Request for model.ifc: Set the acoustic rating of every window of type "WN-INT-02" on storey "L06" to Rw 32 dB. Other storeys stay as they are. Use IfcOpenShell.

First a look at what the model holds.

```python
import ifcopenshell
import ifcopenshell.util.element

model = ifcopenshell.open("model.ifc")
print(model.schema)
storey = next(s for s in model.by_type("IfcBuildingStorey") if s.Name == "L06")
windows = [e for e in ifcopenshell.util.element.get_decomposition(storey) if e.is_a("IfcWindow")]
seen = {}
for e in windows:
    element_type = ifcopenshell.util.element.get_type(e)
    key = (element_type.Name if element_type != e and element_type else None, ifcopenshell.util.element.get_pset(e, "Pset_WindowCommon", "AcousticRating"))
    seen[key] = seen.get(key, 0) + 1
for (name, value), count in sorted(seen.items(), key=str):
    print(count, "x", name, "|", value)
```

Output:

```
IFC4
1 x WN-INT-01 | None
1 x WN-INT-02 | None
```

```python
import ifcopenshell
import ifcopenshell.api.pset
import ifcopenshell.util.element

model = ifcopenshell.open("model.ifc")

storey = next(s for s in model.by_type("IfcBuildingStorey") if s.Name == "L06")
windows = [e for e in ifcopenshell.util.element.get_decomposition(storey) if e.is_a("IfcWindow")]

count = 0
for e in windows:
    element_type = ifcopenshell.util.element.get_type(e)
    if element_type in (None, e) or element_type.Name != "WN-INT-02":
        continue
    # add_pset returns the element's existing set when there is one.
    pset = ifcopenshell.api.pset.add_pset(model, product=e, name="Pset_WindowCommon")
    ifcopenshell.api.pset.edit_pset(model, pset=pset, properties={"AcousticRating": "Rw 32 dB"})
    count += 1

print(count, "windows updated")

model.write("model_v2.ifc")
```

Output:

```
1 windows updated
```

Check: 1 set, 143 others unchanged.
